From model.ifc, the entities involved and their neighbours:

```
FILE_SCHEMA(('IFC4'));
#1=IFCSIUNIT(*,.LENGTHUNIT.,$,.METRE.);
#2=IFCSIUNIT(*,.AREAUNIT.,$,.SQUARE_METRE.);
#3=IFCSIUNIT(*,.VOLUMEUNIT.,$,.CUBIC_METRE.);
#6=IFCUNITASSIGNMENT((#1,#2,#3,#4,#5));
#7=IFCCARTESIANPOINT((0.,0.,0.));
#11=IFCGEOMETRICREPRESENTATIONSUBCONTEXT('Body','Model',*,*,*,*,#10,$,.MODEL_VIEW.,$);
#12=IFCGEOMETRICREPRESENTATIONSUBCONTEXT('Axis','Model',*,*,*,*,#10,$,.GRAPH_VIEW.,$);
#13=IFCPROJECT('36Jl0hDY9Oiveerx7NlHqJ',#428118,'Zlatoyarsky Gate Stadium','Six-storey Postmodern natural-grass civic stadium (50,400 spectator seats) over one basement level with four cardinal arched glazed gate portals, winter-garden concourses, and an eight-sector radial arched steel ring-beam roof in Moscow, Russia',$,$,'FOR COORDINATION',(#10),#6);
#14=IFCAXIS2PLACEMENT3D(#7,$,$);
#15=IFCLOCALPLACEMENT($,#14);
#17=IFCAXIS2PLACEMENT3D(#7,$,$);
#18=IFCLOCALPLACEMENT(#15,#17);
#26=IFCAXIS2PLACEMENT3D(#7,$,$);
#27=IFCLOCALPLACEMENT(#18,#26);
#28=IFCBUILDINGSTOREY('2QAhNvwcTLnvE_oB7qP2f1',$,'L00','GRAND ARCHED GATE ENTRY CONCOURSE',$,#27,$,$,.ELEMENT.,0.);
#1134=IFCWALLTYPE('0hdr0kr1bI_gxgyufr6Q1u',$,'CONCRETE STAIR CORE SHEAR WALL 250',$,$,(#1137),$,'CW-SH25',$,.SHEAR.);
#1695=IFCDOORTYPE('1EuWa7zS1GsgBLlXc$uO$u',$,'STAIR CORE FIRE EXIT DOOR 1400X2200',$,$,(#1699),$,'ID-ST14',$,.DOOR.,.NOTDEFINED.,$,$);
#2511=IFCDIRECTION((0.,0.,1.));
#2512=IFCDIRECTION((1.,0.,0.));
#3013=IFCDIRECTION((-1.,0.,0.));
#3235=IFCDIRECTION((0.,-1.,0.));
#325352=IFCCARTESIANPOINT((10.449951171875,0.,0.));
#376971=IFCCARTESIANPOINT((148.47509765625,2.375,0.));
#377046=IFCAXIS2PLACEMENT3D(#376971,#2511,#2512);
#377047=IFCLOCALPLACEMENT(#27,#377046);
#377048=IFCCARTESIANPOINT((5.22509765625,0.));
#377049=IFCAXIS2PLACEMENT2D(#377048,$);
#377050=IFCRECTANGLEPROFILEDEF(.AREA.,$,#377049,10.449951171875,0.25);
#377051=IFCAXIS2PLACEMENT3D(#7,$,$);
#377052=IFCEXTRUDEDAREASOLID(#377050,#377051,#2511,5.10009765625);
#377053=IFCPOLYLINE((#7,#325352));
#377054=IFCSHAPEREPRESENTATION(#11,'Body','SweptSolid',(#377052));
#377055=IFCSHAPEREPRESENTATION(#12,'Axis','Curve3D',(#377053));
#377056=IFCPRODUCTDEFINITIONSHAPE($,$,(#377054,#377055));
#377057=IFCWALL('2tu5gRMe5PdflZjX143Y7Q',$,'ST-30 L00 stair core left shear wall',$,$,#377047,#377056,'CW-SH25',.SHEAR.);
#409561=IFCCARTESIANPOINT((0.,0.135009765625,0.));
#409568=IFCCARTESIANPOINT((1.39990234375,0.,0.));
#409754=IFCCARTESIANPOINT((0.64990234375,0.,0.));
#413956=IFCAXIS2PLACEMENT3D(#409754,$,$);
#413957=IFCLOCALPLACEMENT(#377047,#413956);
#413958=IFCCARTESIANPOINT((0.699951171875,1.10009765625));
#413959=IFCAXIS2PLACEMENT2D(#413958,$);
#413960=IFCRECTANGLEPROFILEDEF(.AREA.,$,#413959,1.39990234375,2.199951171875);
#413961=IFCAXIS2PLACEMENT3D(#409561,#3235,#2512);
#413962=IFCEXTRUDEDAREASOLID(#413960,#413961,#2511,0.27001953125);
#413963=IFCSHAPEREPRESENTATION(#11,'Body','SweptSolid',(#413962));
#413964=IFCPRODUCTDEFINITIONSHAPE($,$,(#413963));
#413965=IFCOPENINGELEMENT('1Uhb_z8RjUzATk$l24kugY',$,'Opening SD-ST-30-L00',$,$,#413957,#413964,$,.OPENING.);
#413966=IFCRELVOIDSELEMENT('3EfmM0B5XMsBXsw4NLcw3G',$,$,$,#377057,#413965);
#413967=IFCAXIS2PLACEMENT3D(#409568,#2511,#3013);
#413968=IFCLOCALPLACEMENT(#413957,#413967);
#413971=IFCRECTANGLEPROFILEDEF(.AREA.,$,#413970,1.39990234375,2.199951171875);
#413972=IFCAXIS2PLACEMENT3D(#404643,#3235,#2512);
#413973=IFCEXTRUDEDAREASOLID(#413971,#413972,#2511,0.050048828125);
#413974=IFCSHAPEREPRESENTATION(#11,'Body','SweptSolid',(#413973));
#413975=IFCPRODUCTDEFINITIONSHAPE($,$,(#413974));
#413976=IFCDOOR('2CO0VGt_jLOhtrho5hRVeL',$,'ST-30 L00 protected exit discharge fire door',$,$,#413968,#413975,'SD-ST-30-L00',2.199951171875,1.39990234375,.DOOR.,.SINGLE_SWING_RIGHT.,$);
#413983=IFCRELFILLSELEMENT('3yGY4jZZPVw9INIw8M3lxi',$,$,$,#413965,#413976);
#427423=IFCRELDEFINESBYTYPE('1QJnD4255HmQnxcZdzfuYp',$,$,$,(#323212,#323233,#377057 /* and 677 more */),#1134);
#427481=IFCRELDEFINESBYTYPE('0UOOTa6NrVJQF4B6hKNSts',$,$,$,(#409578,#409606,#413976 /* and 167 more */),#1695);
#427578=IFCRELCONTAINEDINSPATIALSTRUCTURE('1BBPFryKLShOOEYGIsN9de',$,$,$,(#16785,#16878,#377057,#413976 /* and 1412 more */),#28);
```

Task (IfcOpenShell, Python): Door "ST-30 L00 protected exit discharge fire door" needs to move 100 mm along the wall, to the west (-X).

```python
import ifcopenshell
import ifcopenshell.api.geometry
import ifcopenshell.util.placement

model = ifcopenshell.open("model.ifc")

door = model.by_guid("2CO0VGt_jLOhtrho5hRVeL")
opening = door.FillsVoids[0].RelatingOpeningElement
wall = opening.VoidsElements[0].RelatingBuildingElement

wall_matrix = ifcopenshell.util.placement.get_local_placement(wall.ObjectPlacement)
shift = wall_matrix[:3, 0] * -0.1
before = ifcopenshell.util.placement.get_local_placement(door.ObjectPlacement)[:3, 3].copy()

# The door is placed relative to its opening, so it follows when the opening moves.
matrix = ifcopenshell.util.placement.get_local_placement(opening.ObjectPlacement)
matrix[:3, 3] += shift
ifcopenshell.api.geometry.edit_object_placement(
    model, product=opening, matrix=matrix, is_si=False, should_transform_children=True
)

after = ifcopenshell.util.placement.get_local_placement(door.ObjectPlacement)[:3, 3]
print("door moved by", (after - before).round(3) + 0.0)

model.write("model_rev.ifc")
```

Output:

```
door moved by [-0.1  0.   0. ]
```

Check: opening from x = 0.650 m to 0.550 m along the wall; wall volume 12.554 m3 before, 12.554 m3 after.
